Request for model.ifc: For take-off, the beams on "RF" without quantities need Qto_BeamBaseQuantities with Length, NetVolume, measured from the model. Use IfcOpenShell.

First a look at what the model holds.

```python
import ifcopenshell
import ifcopenshell.util.element
import ifcopenshell.util.unit

model = ifcopenshell.open("model.ifc")
print(model.schema)
for unit_type in ("LENGTHUNIT", "AREAUNIT", "VOLUMEUNIT"):
    print(unit_type, ifcopenshell.util.unit.calculate_unit_scale(model, unit_type))
storey = next(s for s in model.by_type("IfcBuildingStorey") if s.Name == "RF")
beams = [e for e in ifcopenshell.util.element.get_decomposition(storey) if e.is_a("IfcBeam")]
for e in sorted(beams, key=lambda e: e.id()):
    print(e.id(), e.is_a(), e.Name, list(ifcopenshell.util.element.get_psets(e, qtos_only=True)), sep=" | ")
```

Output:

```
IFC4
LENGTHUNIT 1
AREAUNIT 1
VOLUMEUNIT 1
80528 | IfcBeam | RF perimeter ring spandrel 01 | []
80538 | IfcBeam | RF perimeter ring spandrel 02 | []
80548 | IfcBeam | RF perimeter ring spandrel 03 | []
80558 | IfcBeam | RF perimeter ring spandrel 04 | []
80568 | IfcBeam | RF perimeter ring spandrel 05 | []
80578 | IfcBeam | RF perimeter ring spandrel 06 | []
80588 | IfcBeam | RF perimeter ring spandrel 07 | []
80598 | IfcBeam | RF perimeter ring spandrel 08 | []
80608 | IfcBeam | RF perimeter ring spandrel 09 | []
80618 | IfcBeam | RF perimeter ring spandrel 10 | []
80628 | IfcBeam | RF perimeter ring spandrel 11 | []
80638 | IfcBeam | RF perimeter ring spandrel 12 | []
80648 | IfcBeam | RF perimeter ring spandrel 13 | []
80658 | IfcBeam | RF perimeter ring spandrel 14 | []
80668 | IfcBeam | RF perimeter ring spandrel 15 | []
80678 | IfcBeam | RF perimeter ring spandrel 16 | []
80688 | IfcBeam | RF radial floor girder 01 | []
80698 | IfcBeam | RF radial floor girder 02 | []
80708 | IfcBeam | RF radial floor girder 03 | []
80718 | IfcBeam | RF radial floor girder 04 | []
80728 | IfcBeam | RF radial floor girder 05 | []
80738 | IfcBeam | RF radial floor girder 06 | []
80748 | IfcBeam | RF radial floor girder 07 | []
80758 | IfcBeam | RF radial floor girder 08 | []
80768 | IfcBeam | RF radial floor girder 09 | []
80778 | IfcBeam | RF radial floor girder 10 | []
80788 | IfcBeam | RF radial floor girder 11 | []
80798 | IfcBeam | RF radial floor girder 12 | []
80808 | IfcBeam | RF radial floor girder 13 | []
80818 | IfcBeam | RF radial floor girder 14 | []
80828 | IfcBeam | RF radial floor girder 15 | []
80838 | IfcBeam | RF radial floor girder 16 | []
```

```python
import ifcopenshell
import ifcopenshell.api.pset
import ifcopenshell.geom
import ifcopenshell.util.element
import ifcopenshell.util.shape
import ifcopenshell.util.unit

model = ifcopenshell.open("model.ifc")
unit_scale = ifcopenshell.util.unit.calculate_unit_scale(model)
volume_scale = ifcopenshell.util.unit.calculate_unit_scale(model, "VOLUMEUNIT")
settings = ifcopenshell.geom.settings()

storey = next(s for s in model.by_type("IfcBuildingStorey") if s.Name == "RF")
beams = [e for e in ifcopenshell.util.element.get_decomposition(storey) if e.is_a("IfcBeam")]

for e in sorted(beams, key=lambda e: e.id()):
    if ifcopenshell.util.element.get_psets(e, qtos_only=True, should_inherit=False):
        continue
    # Geometry comes back in metres, in the element's own axes.
    shape = ifcopenshell.geom.create_shape(settings, e)
    values = {
        "Length": ifcopenshell.util.shape.get_max_xyz(shape.geometry) / unit_scale,
        "NetVolume": ifcopenshell.util.shape.get_volume(shape.geometry) / volume_scale,
    }
    qto = ifcopenshell.api.pset.add_qto(model, product=e, name="Qto_BeamBaseQuantities")
    ifcopenshell.api.pset.edit_qto(model, qto=qto, properties=values)
    print(e.id(), {k: round(v, 3) for k, v in values.items()})

model.write("model_rev.ifc")
```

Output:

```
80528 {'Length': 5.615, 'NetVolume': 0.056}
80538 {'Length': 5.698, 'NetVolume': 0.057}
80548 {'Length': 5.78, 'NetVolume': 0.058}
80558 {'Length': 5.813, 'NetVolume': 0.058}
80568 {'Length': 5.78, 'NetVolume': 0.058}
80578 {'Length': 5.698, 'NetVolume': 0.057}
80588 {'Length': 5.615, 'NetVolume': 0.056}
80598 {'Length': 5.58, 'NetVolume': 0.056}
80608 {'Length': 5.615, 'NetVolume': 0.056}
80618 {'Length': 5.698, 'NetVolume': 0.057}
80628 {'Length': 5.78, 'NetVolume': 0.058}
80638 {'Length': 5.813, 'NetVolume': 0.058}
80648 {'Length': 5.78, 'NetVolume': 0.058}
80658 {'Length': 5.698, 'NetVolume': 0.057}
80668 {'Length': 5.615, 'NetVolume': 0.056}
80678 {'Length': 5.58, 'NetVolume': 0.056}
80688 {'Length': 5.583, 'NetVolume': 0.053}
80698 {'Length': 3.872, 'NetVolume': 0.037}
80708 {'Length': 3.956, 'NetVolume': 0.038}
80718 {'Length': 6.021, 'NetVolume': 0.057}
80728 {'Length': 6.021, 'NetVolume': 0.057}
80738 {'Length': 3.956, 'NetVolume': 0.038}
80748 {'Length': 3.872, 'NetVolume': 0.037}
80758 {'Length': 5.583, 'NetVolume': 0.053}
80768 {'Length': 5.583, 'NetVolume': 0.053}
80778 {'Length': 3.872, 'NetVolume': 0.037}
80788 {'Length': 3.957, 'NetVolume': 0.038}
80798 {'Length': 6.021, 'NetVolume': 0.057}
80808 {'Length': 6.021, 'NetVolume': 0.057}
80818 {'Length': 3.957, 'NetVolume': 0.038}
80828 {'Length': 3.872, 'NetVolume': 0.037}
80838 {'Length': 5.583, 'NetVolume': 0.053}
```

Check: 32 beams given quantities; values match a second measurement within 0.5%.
